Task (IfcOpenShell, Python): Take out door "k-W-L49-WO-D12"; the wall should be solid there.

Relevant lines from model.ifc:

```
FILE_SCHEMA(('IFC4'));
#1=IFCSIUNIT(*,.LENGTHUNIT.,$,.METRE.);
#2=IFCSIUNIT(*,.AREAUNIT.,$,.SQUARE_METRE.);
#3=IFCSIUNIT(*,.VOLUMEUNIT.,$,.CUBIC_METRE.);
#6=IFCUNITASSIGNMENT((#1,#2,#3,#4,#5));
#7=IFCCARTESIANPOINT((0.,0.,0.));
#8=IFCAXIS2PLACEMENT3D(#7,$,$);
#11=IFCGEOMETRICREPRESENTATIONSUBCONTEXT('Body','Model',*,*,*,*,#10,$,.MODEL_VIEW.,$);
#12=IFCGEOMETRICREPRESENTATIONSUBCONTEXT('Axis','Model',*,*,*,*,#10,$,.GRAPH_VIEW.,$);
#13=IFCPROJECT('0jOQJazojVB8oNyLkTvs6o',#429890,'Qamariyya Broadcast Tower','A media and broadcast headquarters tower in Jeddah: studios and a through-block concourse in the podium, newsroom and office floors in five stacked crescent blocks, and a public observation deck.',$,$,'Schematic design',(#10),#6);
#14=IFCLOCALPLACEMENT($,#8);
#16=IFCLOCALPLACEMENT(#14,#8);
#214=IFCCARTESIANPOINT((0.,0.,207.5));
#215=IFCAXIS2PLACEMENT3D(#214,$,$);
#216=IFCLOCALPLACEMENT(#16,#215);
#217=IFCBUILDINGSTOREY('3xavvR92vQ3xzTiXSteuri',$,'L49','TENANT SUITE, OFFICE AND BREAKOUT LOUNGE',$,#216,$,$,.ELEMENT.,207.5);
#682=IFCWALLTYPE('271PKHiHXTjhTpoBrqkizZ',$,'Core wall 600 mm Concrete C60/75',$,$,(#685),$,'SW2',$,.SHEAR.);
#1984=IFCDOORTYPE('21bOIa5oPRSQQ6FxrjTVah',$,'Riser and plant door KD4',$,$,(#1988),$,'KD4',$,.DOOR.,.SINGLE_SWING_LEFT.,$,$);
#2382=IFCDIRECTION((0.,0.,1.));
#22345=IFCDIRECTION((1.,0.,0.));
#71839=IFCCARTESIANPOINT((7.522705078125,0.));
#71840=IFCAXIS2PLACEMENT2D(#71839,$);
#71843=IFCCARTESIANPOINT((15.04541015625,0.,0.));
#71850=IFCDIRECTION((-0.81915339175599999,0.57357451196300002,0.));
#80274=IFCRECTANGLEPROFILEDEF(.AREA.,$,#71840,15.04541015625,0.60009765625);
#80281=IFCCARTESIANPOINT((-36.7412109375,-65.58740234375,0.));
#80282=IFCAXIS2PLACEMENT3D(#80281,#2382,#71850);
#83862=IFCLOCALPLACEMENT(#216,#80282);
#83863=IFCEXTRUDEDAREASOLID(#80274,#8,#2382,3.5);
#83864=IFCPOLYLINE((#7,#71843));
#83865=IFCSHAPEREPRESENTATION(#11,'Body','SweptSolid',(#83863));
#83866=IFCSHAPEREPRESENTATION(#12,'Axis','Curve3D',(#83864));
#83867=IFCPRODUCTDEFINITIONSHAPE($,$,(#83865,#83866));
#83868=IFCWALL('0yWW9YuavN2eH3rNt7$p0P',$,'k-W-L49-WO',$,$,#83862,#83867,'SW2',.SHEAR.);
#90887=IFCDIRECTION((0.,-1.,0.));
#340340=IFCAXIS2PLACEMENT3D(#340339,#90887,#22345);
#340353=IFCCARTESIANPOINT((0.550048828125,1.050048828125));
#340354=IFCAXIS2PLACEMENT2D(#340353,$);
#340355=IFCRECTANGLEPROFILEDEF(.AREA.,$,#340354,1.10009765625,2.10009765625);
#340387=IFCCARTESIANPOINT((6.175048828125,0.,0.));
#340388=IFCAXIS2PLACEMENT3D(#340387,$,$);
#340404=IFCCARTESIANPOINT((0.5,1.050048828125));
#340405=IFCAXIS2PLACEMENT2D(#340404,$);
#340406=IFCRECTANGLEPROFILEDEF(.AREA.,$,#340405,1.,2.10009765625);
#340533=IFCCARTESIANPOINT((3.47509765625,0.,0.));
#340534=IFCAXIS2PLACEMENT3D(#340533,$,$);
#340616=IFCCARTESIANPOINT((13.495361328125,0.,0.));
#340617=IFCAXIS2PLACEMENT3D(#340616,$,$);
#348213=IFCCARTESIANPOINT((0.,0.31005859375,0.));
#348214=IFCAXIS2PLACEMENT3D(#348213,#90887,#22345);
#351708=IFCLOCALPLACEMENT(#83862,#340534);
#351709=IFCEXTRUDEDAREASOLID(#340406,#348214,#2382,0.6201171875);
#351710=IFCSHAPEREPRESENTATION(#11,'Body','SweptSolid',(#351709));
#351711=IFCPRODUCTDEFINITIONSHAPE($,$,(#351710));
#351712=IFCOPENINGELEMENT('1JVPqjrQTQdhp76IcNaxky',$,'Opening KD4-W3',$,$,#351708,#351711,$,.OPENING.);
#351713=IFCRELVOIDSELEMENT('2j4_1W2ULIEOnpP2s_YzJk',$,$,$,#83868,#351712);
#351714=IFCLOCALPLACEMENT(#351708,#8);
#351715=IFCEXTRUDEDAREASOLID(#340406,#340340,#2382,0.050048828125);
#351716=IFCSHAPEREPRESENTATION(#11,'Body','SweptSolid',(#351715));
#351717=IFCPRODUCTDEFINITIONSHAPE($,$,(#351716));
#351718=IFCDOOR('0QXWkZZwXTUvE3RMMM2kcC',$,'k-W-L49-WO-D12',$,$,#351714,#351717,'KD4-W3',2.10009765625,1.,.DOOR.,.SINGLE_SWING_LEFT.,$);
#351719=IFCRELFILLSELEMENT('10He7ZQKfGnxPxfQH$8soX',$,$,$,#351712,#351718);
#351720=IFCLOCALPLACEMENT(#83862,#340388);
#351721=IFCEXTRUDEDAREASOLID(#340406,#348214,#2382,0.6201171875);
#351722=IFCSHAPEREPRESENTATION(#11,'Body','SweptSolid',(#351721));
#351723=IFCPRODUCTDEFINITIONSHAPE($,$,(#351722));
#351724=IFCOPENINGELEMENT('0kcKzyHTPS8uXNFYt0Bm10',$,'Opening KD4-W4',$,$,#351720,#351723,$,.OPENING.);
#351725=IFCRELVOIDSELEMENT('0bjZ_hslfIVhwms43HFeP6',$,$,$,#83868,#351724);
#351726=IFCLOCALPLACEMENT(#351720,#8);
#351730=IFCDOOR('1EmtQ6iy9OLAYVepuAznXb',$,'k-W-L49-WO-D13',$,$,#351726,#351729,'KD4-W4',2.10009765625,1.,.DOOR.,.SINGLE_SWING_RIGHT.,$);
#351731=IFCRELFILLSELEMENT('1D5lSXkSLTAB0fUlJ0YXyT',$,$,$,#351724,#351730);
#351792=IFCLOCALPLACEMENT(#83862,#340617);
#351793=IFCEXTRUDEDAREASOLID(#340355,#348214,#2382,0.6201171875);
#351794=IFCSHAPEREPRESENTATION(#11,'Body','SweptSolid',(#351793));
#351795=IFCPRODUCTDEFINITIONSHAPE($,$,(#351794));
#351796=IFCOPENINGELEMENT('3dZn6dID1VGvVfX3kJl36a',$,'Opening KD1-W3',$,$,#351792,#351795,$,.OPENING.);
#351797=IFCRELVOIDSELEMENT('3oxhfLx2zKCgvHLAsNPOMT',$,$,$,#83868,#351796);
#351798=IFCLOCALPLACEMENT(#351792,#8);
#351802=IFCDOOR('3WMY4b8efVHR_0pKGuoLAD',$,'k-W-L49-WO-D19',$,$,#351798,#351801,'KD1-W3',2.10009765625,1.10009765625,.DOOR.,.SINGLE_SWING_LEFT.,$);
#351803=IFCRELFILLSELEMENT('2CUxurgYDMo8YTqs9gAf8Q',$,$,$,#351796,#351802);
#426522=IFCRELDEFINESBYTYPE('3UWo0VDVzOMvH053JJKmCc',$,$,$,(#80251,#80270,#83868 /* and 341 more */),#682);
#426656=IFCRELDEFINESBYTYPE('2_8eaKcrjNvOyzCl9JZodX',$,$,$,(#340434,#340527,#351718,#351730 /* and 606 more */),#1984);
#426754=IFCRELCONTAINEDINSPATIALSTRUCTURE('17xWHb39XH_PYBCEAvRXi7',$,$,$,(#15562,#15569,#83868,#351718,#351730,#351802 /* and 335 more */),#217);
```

```python
import ifcopenshell
import ifcopenshell.api.feature
import ifcopenshell.api.root
import ifcopenshell.geom
import ifcopenshell.util.shape

model = ifcopenshell.open("model.ifc")
settings = ifcopenshell.geom.settings()


def volume(element):
    """Net volume in cubic metres, openings subtracted."""
    shape = ifcopenshell.geom.create_shape(settings, element)
    return ifcopenshell.util.shape.get_volume(shape.geometry)


door = model.by_guid("0QXWkZZwXTUvE3RMMM2kcC")
opening = door.FillsVoids[0].RelatingOpeningElement
wall = opening.VoidsElements[0].RelatingBuildingElement
before = volume(wall)

ifcopenshell.api.root.remove_product(model, product=door)
ifcopenshell.api.feature.remove_feature(model, feature=opening)

after = volume(wall)

print(f"wall volume {before:.3f} -> {after:.3f} m3")

model.write("model_updated.ifc")
```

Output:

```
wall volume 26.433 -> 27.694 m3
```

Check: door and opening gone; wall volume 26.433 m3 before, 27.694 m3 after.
